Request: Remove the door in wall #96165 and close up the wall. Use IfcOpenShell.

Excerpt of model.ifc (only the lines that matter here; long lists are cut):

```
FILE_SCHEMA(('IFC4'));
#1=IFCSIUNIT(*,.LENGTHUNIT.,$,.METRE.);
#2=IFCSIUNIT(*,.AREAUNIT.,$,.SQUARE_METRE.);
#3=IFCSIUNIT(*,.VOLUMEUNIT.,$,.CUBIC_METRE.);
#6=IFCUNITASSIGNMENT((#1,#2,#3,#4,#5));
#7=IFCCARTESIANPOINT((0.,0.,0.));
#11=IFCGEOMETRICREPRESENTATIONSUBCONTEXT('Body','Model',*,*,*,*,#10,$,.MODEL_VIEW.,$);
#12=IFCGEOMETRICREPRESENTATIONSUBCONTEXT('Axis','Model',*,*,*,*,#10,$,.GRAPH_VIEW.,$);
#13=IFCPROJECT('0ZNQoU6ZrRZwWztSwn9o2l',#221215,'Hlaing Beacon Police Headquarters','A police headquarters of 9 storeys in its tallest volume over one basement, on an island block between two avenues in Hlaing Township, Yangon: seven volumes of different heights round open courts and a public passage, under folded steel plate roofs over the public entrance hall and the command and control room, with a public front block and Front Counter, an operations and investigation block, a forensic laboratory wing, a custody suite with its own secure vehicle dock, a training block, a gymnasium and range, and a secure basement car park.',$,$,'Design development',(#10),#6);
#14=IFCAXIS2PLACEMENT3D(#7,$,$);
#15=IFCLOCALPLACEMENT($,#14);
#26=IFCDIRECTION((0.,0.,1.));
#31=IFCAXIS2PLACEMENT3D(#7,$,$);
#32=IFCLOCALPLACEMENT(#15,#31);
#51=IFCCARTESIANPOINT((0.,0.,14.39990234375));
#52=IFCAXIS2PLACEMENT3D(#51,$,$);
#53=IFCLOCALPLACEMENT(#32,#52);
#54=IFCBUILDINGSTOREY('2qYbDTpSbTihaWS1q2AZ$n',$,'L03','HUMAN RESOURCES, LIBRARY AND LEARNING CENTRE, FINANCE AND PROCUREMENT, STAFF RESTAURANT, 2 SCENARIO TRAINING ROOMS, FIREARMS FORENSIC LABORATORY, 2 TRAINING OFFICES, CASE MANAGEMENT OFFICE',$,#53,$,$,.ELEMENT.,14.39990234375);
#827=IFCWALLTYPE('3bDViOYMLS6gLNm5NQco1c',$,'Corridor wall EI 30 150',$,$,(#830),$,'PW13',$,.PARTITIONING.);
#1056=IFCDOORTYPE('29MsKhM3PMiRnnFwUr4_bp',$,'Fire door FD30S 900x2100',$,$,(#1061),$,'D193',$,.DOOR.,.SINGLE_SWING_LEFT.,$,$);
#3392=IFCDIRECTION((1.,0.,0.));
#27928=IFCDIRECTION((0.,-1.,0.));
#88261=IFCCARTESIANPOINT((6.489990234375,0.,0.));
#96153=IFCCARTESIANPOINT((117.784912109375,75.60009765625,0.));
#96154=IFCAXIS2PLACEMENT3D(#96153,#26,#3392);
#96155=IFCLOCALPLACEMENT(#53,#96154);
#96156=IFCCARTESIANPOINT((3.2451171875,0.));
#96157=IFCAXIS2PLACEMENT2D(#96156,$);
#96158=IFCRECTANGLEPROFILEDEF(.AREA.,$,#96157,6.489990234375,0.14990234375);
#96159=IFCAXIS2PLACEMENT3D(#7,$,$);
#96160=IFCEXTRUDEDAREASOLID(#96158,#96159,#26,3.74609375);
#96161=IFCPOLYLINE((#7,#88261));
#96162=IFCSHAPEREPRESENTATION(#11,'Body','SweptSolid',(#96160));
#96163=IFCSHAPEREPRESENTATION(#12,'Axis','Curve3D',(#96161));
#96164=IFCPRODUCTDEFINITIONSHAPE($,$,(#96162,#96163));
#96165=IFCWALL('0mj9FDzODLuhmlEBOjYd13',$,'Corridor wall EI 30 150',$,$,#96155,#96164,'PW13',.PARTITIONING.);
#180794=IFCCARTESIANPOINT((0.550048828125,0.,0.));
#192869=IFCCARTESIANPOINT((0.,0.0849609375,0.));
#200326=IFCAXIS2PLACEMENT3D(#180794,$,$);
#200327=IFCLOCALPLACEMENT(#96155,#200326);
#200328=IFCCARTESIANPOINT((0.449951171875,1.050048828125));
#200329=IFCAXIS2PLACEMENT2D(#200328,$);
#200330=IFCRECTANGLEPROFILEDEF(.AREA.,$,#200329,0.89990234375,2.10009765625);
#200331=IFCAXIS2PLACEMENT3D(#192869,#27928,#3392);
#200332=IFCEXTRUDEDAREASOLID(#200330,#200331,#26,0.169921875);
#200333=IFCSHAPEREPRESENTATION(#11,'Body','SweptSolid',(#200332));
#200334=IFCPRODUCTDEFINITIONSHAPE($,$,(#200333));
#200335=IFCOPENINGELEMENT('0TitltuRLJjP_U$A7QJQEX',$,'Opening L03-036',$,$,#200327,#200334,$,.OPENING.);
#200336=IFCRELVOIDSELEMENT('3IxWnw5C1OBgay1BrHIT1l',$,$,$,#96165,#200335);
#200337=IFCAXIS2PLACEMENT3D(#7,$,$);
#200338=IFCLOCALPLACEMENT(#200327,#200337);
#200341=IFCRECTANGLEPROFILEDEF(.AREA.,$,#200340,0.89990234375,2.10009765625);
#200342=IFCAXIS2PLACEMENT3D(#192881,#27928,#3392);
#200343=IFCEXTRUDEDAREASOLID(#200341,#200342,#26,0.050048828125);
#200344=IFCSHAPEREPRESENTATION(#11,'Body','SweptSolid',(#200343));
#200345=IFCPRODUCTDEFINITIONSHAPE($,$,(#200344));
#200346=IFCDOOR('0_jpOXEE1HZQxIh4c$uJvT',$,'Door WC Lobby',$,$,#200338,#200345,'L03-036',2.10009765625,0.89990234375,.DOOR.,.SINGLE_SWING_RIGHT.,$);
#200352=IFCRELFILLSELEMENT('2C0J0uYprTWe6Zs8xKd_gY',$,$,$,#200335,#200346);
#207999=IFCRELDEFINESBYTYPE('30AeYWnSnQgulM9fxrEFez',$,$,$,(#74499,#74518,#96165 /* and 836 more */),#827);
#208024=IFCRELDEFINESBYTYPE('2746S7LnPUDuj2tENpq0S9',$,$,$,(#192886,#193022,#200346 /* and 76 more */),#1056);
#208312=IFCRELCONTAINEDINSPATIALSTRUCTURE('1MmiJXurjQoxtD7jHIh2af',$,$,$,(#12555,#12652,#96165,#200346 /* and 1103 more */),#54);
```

```python
import ifcopenshell
import ifcopenshell.api.feature
import ifcopenshell.api.root
import ifcopenshell.geom
import ifcopenshell.util.shape

model = ifcopenshell.open("model.ifc")
settings = ifcopenshell.geom.settings()


def volume(element):
    """Net volume in cubic metres, openings subtracted."""
    shape = ifcopenshell.geom.create_shape(settings, element)
    return ifcopenshell.util.shape.get_volume(shape.geometry)


door = model.by_guid("0_jpOXEE1HZQxIh4c$uJvT")
opening = door.FillsVoids[0].RelatingOpeningElement
wall = opening.VoidsElements[0].RelatingBuildingElement
before = volume(wall)

ifcopenshell.api.root.remove_product(model, product=door)
ifcopenshell.api.feature.remove_feature(model, feature=opening)

after = volume(wall)

print(f"wall volume {before:.3f} -> {after:.3f} m3")

model.write("model_rev.ifc")
```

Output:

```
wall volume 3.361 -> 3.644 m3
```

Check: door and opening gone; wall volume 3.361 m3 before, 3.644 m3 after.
